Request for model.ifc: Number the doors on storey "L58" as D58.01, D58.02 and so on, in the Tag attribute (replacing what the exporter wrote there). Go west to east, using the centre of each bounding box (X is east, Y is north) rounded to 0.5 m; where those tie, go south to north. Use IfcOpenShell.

First a look at what the model holds.

```python
import ifcopenshell
import ifcopenshell.util.element
import ifcopenshell.util.placement

model = ifcopenshell.open("model.ifc")
print(model.schema)
storey = next(s for s in model.by_type("IfcBuildingStorey") if s.Name == "L58")
doors = [e for e in ifcopenshell.util.element.get_decomposition(storey) if e.is_a("IfcDoor")]
for e in sorted(doors, key=lambda e: e.id()):
    origin = ifcopenshell.util.placement.get_local_placement(e.ObjectPlacement)[:3, 3]
    print(e.id(), e.Tag, e.Name, origin.round(2) + 0.0, sep=" | ")
```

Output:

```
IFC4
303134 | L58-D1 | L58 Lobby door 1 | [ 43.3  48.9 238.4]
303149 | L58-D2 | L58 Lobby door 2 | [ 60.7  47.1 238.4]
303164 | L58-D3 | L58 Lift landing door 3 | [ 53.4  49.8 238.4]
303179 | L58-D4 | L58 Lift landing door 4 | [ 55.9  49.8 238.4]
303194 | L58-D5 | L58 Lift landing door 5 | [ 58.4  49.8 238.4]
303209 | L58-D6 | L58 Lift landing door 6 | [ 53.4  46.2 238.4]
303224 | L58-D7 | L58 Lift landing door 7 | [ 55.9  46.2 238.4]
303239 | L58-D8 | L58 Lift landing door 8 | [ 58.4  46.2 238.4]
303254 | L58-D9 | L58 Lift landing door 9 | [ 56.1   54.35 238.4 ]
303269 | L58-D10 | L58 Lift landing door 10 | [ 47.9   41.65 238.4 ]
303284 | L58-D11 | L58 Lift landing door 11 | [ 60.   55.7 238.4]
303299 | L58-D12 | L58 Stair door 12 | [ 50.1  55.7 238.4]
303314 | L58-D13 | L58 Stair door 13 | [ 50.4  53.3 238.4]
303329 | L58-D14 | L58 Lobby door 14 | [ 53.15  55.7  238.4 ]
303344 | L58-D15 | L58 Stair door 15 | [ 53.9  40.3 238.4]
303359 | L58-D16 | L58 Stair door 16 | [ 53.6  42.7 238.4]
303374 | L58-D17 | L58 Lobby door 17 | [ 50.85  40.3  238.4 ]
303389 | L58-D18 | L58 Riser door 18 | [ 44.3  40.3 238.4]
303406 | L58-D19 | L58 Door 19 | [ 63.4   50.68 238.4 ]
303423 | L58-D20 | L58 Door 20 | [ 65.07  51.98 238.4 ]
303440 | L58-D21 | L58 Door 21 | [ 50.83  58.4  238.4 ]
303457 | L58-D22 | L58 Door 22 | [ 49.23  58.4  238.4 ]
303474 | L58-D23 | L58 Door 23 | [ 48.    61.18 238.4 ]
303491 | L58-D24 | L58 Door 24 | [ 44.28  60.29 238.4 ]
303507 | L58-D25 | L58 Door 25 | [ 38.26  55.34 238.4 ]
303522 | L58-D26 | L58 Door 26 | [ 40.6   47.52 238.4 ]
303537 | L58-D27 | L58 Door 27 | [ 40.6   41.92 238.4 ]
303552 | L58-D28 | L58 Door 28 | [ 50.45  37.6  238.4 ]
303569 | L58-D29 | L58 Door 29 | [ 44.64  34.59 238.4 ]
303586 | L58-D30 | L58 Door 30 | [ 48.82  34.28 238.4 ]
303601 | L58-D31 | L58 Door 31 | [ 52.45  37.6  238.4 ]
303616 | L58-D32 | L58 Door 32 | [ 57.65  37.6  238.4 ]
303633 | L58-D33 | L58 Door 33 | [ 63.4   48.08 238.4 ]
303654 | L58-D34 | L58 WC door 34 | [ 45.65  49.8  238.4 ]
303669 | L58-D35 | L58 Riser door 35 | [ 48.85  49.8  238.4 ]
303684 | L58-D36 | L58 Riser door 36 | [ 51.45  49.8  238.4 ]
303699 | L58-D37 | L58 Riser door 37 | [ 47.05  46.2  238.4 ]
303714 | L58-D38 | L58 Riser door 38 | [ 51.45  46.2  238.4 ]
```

```python
import ifcopenshell
import ifcopenshell.geom
import ifcopenshell.util.element
import ifcopenshell.util.shape

model = ifcopenshell.open("model.ifc")
settings = ifcopenshell.geom.settings()
settings.set("use-world-coords", True)


def centre(element):
    shape = ifcopenshell.geom.create_shape(settings, element)
    return ifcopenshell.util.shape.get_bbox_centroid(shape.geometry)


storey = next(s for s in model.by_type("IfcBuildingStorey") if s.Name == "L58")
doors = [e for e in ifcopenshell.util.element.get_decomposition(storey) if e.is_a("IfcDoor")]

# Insertion points can sit at a corner or the storey origin, so sort by the geometry (in metres).
centres = {e: centre(e) for e in doors}
doors.sort(key=lambda e: (round(centres[e][0] / 0.5), centres[e][1]))

for i, e in enumerate(doors, start=1):
    number = f"D58.{i:02d}"
    e.Tag = number
    print(e.id(), number)

model.write("model_v2.ifc")
```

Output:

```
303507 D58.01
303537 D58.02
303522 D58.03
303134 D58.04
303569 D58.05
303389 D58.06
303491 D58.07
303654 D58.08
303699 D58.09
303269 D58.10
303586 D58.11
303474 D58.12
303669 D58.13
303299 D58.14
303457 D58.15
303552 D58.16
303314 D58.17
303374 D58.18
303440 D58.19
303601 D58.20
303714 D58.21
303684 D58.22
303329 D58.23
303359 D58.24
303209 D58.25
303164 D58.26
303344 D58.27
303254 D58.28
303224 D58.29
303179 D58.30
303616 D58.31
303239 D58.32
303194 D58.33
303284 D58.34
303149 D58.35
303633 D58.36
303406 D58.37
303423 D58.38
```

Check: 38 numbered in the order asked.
